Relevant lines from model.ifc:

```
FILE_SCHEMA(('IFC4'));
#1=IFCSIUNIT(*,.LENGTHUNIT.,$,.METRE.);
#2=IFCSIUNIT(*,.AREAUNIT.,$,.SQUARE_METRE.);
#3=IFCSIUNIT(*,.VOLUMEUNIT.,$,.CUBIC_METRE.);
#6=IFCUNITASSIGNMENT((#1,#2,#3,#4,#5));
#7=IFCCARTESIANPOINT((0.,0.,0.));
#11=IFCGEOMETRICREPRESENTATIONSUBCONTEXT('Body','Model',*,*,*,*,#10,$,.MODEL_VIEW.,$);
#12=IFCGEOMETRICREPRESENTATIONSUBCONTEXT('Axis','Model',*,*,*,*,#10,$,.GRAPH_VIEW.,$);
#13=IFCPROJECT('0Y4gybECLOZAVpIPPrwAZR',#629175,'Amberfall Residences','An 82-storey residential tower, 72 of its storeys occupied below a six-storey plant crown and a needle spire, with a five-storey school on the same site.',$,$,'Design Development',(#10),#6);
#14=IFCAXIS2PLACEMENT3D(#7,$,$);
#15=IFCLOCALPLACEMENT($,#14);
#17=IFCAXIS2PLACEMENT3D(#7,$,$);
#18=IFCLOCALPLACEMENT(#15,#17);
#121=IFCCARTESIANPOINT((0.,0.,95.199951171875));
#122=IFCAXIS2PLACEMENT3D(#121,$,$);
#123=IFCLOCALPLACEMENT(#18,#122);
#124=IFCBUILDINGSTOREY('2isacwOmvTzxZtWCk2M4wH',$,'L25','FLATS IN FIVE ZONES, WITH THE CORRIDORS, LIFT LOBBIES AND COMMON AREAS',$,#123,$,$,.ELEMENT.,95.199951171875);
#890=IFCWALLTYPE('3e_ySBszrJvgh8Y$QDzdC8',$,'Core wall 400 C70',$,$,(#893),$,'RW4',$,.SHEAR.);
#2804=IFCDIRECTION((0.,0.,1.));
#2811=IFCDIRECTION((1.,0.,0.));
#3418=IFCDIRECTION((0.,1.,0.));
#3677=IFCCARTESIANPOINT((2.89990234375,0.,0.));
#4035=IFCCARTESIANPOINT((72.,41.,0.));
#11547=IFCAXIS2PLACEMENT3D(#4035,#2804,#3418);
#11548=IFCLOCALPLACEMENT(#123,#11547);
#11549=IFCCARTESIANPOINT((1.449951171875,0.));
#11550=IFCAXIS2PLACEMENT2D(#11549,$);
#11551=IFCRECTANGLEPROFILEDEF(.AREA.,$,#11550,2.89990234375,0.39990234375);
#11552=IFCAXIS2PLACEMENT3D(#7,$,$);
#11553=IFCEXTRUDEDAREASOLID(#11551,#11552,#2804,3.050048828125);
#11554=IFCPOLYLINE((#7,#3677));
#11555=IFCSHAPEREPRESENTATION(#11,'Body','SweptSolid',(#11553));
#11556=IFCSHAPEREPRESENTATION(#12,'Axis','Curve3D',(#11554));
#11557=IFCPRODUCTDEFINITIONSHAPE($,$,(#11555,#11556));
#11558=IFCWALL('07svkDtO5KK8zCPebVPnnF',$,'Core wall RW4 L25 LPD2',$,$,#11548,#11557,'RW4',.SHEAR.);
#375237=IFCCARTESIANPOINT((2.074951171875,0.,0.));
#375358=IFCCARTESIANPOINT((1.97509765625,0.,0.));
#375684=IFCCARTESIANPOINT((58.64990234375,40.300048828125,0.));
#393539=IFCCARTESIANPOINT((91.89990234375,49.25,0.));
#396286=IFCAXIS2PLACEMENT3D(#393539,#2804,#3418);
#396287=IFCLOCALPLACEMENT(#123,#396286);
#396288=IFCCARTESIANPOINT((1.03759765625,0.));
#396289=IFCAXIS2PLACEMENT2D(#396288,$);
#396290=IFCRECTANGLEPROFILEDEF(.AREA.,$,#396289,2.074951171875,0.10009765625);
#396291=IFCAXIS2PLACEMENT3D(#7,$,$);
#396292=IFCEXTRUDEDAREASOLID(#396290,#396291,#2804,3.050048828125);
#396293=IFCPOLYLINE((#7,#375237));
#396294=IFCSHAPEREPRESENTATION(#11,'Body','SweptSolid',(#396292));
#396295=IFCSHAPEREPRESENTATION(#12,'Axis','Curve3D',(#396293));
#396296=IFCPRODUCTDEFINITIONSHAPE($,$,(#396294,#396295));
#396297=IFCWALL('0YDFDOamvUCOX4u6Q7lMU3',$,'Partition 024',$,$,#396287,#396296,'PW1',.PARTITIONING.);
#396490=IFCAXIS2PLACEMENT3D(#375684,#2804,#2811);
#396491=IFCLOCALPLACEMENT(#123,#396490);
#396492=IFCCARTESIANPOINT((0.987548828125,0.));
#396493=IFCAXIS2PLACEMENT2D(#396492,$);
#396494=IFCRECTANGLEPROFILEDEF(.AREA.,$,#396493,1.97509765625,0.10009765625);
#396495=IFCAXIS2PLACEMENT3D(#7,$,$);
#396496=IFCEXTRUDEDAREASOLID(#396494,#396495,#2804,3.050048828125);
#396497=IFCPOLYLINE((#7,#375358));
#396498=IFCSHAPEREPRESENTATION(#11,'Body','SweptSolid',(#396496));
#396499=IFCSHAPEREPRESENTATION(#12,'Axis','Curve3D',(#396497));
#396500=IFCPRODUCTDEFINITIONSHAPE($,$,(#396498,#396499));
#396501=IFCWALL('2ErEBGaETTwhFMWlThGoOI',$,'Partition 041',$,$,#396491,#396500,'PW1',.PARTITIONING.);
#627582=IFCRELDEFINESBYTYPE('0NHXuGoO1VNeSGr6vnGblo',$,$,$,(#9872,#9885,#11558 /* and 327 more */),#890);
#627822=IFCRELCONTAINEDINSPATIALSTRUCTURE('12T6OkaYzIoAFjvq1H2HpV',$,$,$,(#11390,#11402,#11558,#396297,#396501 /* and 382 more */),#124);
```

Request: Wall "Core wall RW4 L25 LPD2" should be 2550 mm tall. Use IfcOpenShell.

```python
import ifcopenshell
import ifcopenshell.geom
import ifcopenshell.util.representation
import ifcopenshell.util.shape

model = ifcopenshell.open("model.ifc")
settings = ifcopenshell.geom.settings()


def volume(element):
    """Net volume in cubic metres, openings subtracted."""
    shape = ifcopenshell.geom.create_shape(settings, element)
    return ifcopenshell.util.shape.get_volume(shape.geometry)


wall = model.by_guid("07svkDtO5KK8zCPebVPnnF")
before = volume(wall)

body = ifcopenshell.util.representation.get_representation(wall, "Model", "Body")
solid = body.Items[0]
old_height = solid.Depth
solid.Depth = 2.55
after = volume(wall)

print(f"height {old_height:g} -> {solid.Depth:g}, volume {before:.3f} -> {after:.3f} m3")

model.write("model_updated.ifc")
```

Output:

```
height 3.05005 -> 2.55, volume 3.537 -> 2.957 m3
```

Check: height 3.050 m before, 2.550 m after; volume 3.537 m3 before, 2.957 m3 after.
